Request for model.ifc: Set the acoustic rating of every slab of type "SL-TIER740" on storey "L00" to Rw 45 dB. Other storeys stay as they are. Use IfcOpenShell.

First a look at what the model holds.

```python
import ifcopenshell
import ifcopenshell.util.element

model = ifcopenshell.open("model.ifc")
print(model.schema)
storey = next(s for s in model.by_type("IfcBuildingStorey") if s.Name == "L00")
slabs = [e for e in ifcopenshell.util.element.get_decomposition(storey) if e.is_a("IfcSlab")]
seen = {}
for e in slabs:
    element_type = ifcopenshell.util.element.get_type(e)
    key = (element_type.Name if element_type != e and element_type else None, ifcopenshell.util.element.get_pset(e, "Pset_SlabCommon", "AcousticRating"))
    seen[key] = seen.get(key, 0) + 1
for (name, value), count in sorted(seen.items(), key=str):
    print(count, "x", name, "|", value)
```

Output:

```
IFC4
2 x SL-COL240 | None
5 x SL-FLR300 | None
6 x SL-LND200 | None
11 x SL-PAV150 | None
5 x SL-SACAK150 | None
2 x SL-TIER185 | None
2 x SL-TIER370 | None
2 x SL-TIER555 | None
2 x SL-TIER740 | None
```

```python
import ifcopenshell
import ifcopenshell.api.pset
import ifcopenshell.util.element

model = ifcopenshell.open("model.ifc")

storey = next(s for s in model.by_type("IfcBuildingStorey") if s.Name == "L00")
slabs = [e for e in ifcopenshell.util.element.get_decomposition(storey) if e.is_a("IfcSlab")]

count = 0
for e in slabs:
    element_type = ifcopenshell.util.element.get_type(e)
    if element_type in (None, e) or element_type.Name != "SL-TIER740":
        continue
    # add_pset returns the element's existing set when there is one.
    pset = ifcopenshell.api.pset.add_pset(model, product=e, name="Pset_SlabCommon")
    ifcopenshell.api.pset.edit_pset(model, pset=pset, properties={"AcousticRating": "Rw 45 dB"})
    count += 1

print(count, "slabs updated")

model.write("model_edited.ifc")
```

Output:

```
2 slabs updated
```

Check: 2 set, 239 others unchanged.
